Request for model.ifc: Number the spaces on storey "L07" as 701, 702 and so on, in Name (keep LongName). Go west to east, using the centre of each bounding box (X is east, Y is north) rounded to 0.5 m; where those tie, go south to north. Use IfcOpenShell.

First a look at what the model holds.

```python
import ifcopenshell
import ifcopenshell.util.element
import ifcopenshell.util.placement

model = ifcopenshell.open("model.ifc")
print(model.schema)
storey = next(s for s in model.by_type("IfcBuildingStorey") if s.Name == "L07")
spaces = [e for e in ifcopenshell.util.element.get_decomposition(storey) if e.is_a("IfcSpace")]
for e in sorted(spaces, key=lambda e: e.id()):
    origin = ifcopenshell.util.placement.get_local_placement(e.ObjectPlacement)[:3, 3]
    print(e.id(), e.Name, e.LongName, origin.round(2) + 0.0, sep=" | ")
```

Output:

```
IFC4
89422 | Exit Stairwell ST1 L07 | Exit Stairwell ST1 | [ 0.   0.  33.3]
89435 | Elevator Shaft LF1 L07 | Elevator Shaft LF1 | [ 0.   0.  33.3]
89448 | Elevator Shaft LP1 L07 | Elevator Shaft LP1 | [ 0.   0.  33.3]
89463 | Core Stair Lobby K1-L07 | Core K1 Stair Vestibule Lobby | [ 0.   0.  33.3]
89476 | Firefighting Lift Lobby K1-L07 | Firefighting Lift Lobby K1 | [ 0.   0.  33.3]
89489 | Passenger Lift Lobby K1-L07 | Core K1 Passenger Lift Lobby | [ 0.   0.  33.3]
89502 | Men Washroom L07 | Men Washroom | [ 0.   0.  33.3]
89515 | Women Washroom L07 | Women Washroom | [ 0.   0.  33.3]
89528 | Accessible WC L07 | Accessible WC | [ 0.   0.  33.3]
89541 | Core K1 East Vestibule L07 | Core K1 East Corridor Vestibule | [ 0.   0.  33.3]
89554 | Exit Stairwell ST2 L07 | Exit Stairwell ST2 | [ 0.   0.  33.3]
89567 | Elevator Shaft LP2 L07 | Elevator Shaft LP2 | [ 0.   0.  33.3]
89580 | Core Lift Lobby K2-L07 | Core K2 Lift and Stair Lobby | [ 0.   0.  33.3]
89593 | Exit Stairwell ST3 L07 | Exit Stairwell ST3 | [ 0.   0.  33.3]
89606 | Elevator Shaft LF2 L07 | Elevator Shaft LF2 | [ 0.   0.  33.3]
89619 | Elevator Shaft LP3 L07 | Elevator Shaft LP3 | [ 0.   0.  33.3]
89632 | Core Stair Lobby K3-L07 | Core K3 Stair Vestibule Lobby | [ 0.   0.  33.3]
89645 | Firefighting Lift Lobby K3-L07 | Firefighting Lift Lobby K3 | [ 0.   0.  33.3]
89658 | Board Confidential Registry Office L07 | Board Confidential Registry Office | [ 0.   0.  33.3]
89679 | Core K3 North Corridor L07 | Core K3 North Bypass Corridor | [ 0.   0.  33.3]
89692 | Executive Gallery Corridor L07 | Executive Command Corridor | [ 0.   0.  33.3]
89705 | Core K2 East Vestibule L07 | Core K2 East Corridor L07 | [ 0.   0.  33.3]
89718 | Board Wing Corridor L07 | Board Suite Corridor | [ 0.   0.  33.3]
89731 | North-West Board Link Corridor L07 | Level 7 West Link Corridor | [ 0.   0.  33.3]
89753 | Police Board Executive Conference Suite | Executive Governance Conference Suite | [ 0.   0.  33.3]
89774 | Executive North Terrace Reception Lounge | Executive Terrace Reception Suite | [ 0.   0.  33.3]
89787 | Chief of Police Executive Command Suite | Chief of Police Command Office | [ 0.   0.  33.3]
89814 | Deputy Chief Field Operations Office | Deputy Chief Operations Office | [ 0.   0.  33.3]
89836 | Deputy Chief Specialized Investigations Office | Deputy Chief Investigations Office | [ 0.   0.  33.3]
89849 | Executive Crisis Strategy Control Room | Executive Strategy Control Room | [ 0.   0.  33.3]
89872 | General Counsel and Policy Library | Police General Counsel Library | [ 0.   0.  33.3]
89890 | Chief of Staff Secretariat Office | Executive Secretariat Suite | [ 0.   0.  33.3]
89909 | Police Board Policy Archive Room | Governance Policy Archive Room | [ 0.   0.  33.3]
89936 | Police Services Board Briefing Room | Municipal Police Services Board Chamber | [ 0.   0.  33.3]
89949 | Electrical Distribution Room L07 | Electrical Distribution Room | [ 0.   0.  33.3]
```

```python
import ifcopenshell
import ifcopenshell.geom
import ifcopenshell.util.element
import ifcopenshell.util.shape

model = ifcopenshell.open("model.ifc")
settings = ifcopenshell.geom.settings()
settings.set("use-world-coords", True)


def centre(element):
    shape = ifcopenshell.geom.create_shape(settings, element)
    return ifcopenshell.util.shape.get_bbox_centroid(shape.geometry)


storey = next(s for s in model.by_type("IfcBuildingStorey") if s.Name == "L07")
spaces = [e for e in ifcopenshell.util.element.get_decomposition(storey) if e.is_a("IfcSpace")]

# Insertion points can sit at a corner or the storey origin, so sort by the geometry (in metres).
centres = {e: centre(e) for e in spaces}
spaces.sort(key=lambda e: (round(centres[e][0] / 0.5), centres[e][1]))

for i, e in enumerate(spaces, start=1):
    number = f"7{i:02d}"
    e.Name = number
    print(e.id(), number)

model.write("model_edited.ifc")
```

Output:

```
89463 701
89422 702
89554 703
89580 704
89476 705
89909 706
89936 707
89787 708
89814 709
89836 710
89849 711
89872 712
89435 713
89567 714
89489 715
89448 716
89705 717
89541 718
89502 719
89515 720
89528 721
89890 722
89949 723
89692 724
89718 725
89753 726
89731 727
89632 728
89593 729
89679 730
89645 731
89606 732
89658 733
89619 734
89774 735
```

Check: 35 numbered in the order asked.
